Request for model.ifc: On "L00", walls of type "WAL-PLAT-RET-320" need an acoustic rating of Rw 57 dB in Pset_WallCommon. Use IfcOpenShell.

First a look at what the model holds.

```python
import ifcopenshell
import ifcopenshell.util.element

model = ifcopenshell.open("model.ifc")
print(model.schema)
storey = next(s for s in model.by_type("IfcBuildingStorey") if s.Name == "L00")
walls = [e for e in ifcopenshell.util.element.get_decomposition(storey) if e.is_a("IfcWall")]
seen = {}
for e in walls:
    element_type = ifcopenshell.util.element.get_type(e)
    key = (element_type.Name if element_type != e and element_type else None, ifcopenshell.util.element.get_pset(e, "Pset_WallCommon", "AcousticRating"))
    seen[key] = seen.get(key, 0) + 1
for (name, value), count in sorted(seen.items(), key=str):
    print(count, "x", name, "|", value)
```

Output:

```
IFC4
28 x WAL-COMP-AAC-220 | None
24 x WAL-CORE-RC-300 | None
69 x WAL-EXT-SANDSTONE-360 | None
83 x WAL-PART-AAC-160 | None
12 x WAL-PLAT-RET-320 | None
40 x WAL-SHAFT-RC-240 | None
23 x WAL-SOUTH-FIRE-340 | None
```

```python
import ifcopenshell
import ifcopenshell.api.pset
import ifcopenshell.util.element

model = ifcopenshell.open("model.ifc")

storey = next(s for s in model.by_type("IfcBuildingStorey") if s.Name == "L00")
walls = [e for e in ifcopenshell.util.element.get_decomposition(storey) if e.is_a("IfcWall")]

count = 0
for e in walls:
    element_type = ifcopenshell.util.element.get_type(e)
    if element_type in (None, e) or element_type.Name != "WAL-PLAT-RET-320":
        continue
    # add_pset returns the element's existing set when there is one.
    pset = ifcopenshell.api.pset.add_pset(model, product=e, name="Pset_WallCommon")
    ifcopenshell.api.pset.edit_pset(model, pset=pset, properties={"AcousticRating": "Rw 57 dB"})
    count += 1

print(count, "walls updated")

model.write("model_v2.ifc")
```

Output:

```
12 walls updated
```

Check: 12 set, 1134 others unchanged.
